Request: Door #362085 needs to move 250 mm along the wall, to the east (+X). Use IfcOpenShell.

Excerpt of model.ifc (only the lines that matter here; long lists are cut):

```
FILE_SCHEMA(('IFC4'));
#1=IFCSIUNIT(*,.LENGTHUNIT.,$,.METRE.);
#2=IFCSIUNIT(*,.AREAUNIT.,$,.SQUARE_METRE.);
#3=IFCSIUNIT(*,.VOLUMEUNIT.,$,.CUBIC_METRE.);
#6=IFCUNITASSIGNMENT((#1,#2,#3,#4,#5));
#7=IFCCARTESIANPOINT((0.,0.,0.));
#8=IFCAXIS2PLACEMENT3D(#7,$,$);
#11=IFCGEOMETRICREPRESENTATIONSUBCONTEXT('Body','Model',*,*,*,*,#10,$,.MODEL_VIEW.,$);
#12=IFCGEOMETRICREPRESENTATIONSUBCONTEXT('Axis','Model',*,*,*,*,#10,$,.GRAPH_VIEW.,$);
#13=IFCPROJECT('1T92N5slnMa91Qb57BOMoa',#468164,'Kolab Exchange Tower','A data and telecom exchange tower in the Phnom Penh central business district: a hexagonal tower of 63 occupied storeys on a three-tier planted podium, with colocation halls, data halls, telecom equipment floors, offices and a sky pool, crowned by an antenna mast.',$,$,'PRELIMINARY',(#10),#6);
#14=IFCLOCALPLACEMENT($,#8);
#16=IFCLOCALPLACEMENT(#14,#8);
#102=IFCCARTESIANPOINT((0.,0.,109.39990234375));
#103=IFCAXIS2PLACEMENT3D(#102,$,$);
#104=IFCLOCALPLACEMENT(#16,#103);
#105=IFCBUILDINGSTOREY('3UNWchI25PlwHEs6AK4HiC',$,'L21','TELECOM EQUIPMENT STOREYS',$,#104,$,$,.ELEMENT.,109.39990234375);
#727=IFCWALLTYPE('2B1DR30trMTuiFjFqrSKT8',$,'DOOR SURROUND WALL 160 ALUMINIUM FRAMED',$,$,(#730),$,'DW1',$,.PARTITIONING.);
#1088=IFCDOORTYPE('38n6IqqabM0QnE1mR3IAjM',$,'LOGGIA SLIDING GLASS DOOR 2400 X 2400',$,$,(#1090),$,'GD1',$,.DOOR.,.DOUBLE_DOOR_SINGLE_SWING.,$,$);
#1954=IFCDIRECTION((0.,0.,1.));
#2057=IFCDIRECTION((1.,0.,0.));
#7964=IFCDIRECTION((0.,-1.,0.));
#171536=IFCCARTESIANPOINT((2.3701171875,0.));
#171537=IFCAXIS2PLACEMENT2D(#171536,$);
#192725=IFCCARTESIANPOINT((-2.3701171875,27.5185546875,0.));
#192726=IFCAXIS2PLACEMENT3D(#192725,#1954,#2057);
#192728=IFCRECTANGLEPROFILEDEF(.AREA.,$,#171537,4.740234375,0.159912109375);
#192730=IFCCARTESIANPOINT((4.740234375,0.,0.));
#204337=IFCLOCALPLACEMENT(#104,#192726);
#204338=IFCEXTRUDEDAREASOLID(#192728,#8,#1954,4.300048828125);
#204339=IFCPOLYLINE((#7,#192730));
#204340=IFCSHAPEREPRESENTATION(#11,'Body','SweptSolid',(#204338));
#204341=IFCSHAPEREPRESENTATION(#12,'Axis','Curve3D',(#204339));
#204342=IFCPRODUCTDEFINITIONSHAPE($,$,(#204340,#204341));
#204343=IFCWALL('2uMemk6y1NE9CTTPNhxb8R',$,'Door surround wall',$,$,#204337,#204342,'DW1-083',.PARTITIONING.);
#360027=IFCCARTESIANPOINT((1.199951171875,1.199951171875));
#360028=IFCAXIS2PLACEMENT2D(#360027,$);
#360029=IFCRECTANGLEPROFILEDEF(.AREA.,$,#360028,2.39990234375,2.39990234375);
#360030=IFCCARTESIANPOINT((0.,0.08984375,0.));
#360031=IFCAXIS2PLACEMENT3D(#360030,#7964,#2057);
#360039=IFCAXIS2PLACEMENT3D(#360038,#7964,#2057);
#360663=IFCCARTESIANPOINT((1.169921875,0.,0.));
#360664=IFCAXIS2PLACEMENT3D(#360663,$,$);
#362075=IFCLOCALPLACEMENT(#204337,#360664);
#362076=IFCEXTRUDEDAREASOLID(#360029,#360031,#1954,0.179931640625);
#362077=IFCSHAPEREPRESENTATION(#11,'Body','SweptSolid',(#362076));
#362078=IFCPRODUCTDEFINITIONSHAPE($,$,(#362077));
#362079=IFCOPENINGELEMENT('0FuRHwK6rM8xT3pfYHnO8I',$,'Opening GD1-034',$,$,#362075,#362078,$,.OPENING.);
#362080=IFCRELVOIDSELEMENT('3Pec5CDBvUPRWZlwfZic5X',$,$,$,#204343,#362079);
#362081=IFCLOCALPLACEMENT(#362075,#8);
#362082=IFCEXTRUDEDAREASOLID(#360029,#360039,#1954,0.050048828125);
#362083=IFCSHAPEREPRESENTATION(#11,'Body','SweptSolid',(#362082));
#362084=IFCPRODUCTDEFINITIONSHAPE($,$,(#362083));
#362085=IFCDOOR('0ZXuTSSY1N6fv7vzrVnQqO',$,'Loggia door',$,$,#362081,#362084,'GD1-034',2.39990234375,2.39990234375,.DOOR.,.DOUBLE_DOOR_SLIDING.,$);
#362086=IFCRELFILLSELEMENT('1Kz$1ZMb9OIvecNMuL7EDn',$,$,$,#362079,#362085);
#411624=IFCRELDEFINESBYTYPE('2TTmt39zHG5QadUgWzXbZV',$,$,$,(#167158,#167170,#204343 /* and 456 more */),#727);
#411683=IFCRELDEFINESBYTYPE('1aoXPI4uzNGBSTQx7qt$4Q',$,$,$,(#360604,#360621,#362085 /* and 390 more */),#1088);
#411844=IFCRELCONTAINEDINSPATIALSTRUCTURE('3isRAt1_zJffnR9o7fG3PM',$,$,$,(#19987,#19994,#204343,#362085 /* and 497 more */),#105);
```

```python
import ifcopenshell
import ifcopenshell.api.geometry
import ifcopenshell.util.placement
import ifcopenshell.util.unit

model = ifcopenshell.open("model.ifc")
unit_scale = ifcopenshell.util.unit.calculate_unit_scale(model)

door = model.by_guid("0ZXuTSSY1N6fv7vzrVnQqO")
opening = door.FillsVoids[0].RelatingOpeningElement
wall = opening.VoidsElements[0].RelatingBuildingElement

wall_matrix = ifcopenshell.util.placement.get_local_placement(wall.ObjectPlacement)
shift = wall_matrix[:3, 0] * 0.25 / unit_scale
before = ifcopenshell.util.placement.get_local_placement(door.ObjectPlacement)[:3, 3].copy()

# The door is placed relative to its opening, so it follows when the opening moves.
matrix = ifcopenshell.util.placement.get_local_placement(opening.ObjectPlacement)
matrix[:3, 3] += shift
ifcopenshell.api.geometry.edit_object_placement(
    model, product=opening, matrix=matrix, is_si=False, should_transform_children=True
)

after = ifcopenshell.util.placement.get_local_placement(door.ObjectPlacement)[:3, 3]
print("door moved by", (after - before).round(3) + 0.0)

model.write("model-out.ifc")
```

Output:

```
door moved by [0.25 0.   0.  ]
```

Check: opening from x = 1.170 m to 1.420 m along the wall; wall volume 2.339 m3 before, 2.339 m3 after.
